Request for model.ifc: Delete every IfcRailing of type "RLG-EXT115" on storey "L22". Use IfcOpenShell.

First a look at what the model holds.

```python
import ifcopenshell
import ifcopenshell.util.element

model = ifcopenshell.open("model.ifc")
print(model.schema)
storey = next(s for s in model.by_type("IfcBuildingStorey") if s.Name == "L22")
railings = [e for e in ifcopenshell.util.element.get_decomposition(storey) if e.is_a("IfcRailing")]
seen = {}
for e in railings:
    element_type = ifcopenshell.util.element.get_type(e)
    name = element_type.Name if element_type not in (None, e) else None
    seen[name] = seen.get(name, 0) + 1
for name, count in sorted(seen.items(), key=str):
    print(count, "x", name)
```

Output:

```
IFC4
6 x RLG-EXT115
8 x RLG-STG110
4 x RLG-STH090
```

```python
import ifcopenshell
import ifcopenshell.api.root
import ifcopenshell.util.element

model = ifcopenshell.open("model.ifc")

storey = next(s for s in model.by_type("IfcBuildingStorey") if s.Name == "L22")
railings = [e for e in ifcopenshell.util.element.get_decomposition(storey) if e.is_a("IfcRailing")]
targets = [e for e in railings if (t := ifcopenshell.util.element.get_type(e)) not in (None, e) and t.Name == "RLG-EXT115"]

for e in targets:
    ifcopenshell.api.root.remove_product(model, product=e)
print(len(targets), "removed")

model.write("model_edited.ifc")
```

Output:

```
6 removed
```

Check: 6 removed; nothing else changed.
